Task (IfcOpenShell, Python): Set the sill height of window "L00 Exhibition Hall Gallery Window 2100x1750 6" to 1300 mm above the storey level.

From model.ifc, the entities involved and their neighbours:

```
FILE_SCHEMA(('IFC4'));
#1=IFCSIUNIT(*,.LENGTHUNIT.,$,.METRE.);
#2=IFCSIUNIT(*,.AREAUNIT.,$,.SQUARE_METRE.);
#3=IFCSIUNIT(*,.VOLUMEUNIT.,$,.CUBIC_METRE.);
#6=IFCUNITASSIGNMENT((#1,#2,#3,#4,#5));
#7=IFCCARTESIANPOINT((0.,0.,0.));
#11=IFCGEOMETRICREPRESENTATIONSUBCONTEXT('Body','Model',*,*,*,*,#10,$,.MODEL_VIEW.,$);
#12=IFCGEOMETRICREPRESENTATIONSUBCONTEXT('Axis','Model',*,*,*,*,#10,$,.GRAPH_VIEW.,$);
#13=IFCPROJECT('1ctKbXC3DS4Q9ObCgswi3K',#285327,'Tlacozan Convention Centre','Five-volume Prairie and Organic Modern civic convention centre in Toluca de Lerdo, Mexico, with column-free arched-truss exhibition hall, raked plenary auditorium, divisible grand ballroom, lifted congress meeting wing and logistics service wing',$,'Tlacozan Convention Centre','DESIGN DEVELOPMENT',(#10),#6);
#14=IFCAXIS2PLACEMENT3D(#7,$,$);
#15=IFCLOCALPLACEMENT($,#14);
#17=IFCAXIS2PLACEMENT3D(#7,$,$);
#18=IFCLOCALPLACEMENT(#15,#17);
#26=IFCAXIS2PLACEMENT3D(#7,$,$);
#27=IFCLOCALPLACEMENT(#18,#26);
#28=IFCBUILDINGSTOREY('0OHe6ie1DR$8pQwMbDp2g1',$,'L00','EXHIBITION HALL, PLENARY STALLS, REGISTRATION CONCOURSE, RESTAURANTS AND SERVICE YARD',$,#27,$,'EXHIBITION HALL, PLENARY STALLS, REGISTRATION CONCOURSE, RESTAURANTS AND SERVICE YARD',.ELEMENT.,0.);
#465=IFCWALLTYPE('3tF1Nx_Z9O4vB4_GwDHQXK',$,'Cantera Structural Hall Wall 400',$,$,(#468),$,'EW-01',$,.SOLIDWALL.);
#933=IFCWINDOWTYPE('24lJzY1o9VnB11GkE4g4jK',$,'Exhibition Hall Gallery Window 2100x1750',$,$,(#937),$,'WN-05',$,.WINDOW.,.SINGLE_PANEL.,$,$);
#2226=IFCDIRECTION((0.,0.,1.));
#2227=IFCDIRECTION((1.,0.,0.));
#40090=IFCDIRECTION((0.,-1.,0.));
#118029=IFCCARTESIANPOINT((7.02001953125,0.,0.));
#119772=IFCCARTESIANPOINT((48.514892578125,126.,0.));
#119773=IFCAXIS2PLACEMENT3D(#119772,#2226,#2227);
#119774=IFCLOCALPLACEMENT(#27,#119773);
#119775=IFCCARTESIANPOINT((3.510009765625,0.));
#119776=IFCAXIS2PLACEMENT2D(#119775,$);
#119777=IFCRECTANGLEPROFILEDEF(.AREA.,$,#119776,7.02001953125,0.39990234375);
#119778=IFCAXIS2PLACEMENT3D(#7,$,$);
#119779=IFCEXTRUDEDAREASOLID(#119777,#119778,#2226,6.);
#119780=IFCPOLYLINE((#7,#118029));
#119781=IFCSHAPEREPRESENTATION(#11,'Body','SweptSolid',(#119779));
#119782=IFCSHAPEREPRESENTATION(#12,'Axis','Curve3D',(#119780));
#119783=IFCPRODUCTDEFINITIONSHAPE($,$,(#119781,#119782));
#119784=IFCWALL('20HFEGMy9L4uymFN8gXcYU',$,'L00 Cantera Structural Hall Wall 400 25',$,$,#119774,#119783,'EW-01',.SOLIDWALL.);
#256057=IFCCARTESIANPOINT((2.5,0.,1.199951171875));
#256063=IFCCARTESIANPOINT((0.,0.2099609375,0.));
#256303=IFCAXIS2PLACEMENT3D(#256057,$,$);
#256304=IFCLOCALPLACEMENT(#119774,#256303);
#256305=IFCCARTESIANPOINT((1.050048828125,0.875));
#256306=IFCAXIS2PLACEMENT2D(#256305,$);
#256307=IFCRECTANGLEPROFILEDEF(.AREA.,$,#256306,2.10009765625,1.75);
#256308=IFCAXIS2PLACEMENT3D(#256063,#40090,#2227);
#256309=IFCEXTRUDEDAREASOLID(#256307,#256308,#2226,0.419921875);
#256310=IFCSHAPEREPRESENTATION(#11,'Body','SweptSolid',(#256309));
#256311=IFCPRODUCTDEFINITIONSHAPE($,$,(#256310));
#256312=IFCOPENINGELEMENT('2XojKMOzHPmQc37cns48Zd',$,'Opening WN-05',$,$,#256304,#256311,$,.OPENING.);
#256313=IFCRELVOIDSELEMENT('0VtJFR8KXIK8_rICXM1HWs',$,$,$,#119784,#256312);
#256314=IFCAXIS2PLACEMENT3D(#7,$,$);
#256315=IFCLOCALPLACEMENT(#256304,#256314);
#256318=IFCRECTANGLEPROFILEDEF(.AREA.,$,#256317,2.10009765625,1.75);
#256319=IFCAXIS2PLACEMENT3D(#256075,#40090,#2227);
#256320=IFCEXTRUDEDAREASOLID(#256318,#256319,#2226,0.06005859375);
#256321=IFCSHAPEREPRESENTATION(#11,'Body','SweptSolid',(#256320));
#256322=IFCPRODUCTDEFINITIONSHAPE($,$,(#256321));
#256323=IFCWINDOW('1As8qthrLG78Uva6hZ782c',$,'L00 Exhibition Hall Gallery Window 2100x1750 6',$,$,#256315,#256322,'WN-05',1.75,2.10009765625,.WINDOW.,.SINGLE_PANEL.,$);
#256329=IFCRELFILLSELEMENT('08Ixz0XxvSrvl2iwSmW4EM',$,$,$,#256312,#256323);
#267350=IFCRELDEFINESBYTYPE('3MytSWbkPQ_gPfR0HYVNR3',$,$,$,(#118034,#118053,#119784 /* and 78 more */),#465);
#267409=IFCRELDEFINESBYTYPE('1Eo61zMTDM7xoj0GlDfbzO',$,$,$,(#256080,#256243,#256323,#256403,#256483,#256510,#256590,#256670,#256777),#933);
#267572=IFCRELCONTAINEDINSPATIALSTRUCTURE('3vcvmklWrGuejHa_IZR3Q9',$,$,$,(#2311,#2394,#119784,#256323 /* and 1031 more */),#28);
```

```python
import numpy as np
import ifcopenshell
import ifcopenshell.api.geometry
import ifcopenshell.geom
import ifcopenshell.util.element
import ifcopenshell.util.placement
import ifcopenshell.util.shape
import ifcopenshell.util.unit

model = ifcopenshell.open("model.ifc")
unit_scale = ifcopenshell.util.unit.calculate_unit_scale(model)

window = model.by_id(256323)
opening = window.FillsVoids[0].RelatingOpeningElement
storey = ifcopenshell.util.element.get_container(window, ifc_class="IfcBuildingStorey")
level = ifcopenshell.util.placement.get_local_placement(storey.ObjectPlacement)[2, 3]

# The opening's origin need not be at the sill, so measure its lowest point.
shape = ifcopenshell.geom.create_shape(ifcopenshell.geom.settings(), opening)
bottom = ifcopenshell.util.shape.get_shape_bottom_elevation(shape, shape.geometry) / unit_scale
dz = level + 1.3 / unit_scale - bottom

shift = np.array([0.0, 0.0, dz])
# The window is placed relative to its opening, so it follows when the opening moves.
matrix = ifcopenshell.util.placement.get_local_placement(opening.ObjectPlacement)
matrix[:3, 3] += shift
ifcopenshell.api.geometry.edit_object_placement(
    model, product=opening, matrix=matrix, is_si=False, should_transform_children=True
)

print(f"moved by {dz * unit_scale:+.3f} m")

model.write("model-out.ifc")
```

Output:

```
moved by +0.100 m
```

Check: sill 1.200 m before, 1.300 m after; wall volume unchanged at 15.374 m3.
